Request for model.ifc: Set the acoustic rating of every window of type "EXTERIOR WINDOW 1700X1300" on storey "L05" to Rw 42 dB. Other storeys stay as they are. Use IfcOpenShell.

First a look at what the model holds.

```python
import ifcopenshell
import ifcopenshell.util.element

model = ifcopenshell.open("model.ifc")
print(model.schema)
storey = next(s for s in model.by_type("IfcBuildingStorey") if s.Name == "L05")
windows = [e for e in ifcopenshell.util.element.get_decomposition(storey) if e.is_a("IfcWindow")]
seen = {}
for e in windows:
    element_type = ifcopenshell.util.element.get_type(e)
    key = (element_type.Name if element_type != e and element_type else None, ifcopenshell.util.element.get_pset(e, "Pset_WindowCommon", "AcousticRating"))
    seen[key] = seen.get(key, 0) + 1
for (name, value), count in sorted(seen.items(), key=str):
    print(count, "x", name, "|", value)
```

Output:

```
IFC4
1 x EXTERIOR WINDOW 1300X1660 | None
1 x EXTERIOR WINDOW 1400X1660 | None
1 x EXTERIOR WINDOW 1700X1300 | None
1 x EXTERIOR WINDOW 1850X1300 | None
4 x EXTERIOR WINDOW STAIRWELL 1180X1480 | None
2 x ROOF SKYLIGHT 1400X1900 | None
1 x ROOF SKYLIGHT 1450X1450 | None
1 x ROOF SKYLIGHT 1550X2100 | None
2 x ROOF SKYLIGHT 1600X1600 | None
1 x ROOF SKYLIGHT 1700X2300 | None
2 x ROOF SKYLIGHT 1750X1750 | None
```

```python
import ifcopenshell
import ifcopenshell.api.pset
import ifcopenshell.util.element

model = ifcopenshell.open("model.ifc")

storey = next(s for s in model.by_type("IfcBuildingStorey") if s.Name == "L05")
windows = [e for e in ifcopenshell.util.element.get_decomposition(storey) if e.is_a("IfcWindow")]

count = 0
for e in windows:
    element_type = ifcopenshell.util.element.get_type(e)
    if element_type in (None, e) or element_type.Name != "EXTERIOR WINDOW 1700X1300":
        continue
    # add_pset returns the element's existing set when there is one.
    pset = ifcopenshell.api.pset.add_pset(model, product=e, name="Pset_WindowCommon")
    ifcopenshell.api.pset.edit_pset(model, pset=pset, properties={"AcousticRating": "Rw 42 dB"})
    count += 1

print(count, "windows updated")

model.write("model_updated.ifc")
```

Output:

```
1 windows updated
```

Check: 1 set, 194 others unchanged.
